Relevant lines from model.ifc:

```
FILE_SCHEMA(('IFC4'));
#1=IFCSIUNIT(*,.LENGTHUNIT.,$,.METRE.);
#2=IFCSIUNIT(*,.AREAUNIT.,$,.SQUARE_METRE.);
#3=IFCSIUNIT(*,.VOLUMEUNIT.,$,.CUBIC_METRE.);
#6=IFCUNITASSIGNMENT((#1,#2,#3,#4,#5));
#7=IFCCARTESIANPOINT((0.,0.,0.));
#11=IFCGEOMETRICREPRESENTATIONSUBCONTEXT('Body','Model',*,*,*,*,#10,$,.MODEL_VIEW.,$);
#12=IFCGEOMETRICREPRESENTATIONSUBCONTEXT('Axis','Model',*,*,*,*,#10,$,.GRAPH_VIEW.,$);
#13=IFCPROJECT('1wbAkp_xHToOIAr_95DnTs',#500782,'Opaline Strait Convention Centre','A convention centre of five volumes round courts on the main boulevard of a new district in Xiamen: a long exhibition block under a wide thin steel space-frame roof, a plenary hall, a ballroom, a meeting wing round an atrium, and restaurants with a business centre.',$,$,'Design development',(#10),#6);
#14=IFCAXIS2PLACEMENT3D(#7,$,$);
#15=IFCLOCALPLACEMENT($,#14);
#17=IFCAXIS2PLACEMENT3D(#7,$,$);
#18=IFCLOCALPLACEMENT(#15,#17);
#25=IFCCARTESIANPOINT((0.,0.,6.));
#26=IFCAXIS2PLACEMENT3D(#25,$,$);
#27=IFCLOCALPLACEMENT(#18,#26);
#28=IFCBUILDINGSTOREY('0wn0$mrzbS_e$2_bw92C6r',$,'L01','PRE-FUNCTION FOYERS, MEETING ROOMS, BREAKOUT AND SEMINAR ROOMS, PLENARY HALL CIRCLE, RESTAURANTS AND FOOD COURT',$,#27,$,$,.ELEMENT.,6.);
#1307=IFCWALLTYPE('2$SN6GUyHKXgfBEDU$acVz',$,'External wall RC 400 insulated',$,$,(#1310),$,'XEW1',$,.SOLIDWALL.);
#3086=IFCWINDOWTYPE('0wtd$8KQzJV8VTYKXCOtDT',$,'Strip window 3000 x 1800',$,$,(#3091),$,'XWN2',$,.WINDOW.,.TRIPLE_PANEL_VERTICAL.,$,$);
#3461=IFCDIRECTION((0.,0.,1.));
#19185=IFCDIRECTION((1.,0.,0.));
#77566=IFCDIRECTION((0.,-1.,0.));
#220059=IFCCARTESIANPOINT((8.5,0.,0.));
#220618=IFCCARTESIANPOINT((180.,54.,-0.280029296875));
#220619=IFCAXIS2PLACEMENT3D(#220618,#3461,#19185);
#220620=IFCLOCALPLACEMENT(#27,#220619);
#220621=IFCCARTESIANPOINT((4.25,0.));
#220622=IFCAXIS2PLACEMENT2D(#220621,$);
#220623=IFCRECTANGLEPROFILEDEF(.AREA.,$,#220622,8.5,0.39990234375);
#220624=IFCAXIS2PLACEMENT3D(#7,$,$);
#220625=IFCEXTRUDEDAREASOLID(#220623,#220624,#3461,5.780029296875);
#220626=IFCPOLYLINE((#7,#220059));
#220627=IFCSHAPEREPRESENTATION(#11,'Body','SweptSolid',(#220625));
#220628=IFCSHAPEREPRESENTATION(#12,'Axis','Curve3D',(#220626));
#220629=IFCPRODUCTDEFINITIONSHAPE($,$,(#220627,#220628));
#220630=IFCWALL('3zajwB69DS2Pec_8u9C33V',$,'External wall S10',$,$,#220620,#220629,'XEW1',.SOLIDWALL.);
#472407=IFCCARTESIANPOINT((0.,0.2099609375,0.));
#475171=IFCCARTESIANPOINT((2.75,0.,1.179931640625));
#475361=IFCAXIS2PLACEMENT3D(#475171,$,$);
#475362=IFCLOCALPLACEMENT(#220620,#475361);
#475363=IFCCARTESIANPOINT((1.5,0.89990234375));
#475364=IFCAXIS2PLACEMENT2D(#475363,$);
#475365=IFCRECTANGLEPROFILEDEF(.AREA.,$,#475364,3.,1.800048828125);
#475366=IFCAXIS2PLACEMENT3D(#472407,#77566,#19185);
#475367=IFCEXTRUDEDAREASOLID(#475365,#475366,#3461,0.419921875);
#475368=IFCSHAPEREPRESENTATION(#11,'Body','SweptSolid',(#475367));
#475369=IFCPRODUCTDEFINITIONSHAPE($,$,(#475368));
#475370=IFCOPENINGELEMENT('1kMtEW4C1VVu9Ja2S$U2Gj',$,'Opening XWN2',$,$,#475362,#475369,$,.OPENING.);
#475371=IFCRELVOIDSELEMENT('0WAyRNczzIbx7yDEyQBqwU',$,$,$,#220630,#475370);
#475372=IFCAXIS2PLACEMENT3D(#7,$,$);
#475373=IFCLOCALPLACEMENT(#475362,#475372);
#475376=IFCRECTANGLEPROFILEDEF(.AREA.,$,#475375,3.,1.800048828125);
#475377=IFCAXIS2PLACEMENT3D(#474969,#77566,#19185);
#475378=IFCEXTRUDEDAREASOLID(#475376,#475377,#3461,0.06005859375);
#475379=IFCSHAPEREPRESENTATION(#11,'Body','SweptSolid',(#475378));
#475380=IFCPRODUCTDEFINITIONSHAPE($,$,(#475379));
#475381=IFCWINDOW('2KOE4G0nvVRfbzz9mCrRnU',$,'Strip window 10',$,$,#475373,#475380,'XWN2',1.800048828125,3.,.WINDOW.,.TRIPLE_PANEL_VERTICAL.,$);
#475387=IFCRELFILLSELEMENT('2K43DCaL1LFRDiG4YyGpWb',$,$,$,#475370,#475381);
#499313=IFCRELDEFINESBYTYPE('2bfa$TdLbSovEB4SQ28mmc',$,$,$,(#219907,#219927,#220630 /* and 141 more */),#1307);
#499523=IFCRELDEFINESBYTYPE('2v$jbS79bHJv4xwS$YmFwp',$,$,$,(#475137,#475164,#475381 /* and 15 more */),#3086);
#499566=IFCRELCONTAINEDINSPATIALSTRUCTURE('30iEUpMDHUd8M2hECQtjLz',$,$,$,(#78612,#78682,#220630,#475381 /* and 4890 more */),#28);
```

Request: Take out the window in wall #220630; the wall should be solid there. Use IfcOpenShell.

```python
import ifcopenshell
import ifcopenshell.api.feature
import ifcopenshell.api.root
import ifcopenshell.geom
import ifcopenshell.util.shape

model = ifcopenshell.open("model.ifc")
settings = ifcopenshell.geom.settings()


def volume(element):
    """Net volume in cubic metres, openings subtracted."""
    shape = ifcopenshell.geom.create_shape(settings, element)
    return ifcopenshell.util.shape.get_volume(shape.geometry)


window = model.by_guid("2KOE4G0nvVRfbzz9mCrRnU")
opening = window.FillsVoids[0].RelatingOpeningElement
wall = opening.VoidsElements[0].RelatingBuildingElement
before = volume(wall)

ifcopenshell.api.root.remove_product(model, product=window)
ifcopenshell.api.feature.remove_feature(model, feature=opening)

after = volume(wall)

print(f"wall volume {before:.3f} -> {after:.3f} m3")

model.write("model_edited.ifc")
```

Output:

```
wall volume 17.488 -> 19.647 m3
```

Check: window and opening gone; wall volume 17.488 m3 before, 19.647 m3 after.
